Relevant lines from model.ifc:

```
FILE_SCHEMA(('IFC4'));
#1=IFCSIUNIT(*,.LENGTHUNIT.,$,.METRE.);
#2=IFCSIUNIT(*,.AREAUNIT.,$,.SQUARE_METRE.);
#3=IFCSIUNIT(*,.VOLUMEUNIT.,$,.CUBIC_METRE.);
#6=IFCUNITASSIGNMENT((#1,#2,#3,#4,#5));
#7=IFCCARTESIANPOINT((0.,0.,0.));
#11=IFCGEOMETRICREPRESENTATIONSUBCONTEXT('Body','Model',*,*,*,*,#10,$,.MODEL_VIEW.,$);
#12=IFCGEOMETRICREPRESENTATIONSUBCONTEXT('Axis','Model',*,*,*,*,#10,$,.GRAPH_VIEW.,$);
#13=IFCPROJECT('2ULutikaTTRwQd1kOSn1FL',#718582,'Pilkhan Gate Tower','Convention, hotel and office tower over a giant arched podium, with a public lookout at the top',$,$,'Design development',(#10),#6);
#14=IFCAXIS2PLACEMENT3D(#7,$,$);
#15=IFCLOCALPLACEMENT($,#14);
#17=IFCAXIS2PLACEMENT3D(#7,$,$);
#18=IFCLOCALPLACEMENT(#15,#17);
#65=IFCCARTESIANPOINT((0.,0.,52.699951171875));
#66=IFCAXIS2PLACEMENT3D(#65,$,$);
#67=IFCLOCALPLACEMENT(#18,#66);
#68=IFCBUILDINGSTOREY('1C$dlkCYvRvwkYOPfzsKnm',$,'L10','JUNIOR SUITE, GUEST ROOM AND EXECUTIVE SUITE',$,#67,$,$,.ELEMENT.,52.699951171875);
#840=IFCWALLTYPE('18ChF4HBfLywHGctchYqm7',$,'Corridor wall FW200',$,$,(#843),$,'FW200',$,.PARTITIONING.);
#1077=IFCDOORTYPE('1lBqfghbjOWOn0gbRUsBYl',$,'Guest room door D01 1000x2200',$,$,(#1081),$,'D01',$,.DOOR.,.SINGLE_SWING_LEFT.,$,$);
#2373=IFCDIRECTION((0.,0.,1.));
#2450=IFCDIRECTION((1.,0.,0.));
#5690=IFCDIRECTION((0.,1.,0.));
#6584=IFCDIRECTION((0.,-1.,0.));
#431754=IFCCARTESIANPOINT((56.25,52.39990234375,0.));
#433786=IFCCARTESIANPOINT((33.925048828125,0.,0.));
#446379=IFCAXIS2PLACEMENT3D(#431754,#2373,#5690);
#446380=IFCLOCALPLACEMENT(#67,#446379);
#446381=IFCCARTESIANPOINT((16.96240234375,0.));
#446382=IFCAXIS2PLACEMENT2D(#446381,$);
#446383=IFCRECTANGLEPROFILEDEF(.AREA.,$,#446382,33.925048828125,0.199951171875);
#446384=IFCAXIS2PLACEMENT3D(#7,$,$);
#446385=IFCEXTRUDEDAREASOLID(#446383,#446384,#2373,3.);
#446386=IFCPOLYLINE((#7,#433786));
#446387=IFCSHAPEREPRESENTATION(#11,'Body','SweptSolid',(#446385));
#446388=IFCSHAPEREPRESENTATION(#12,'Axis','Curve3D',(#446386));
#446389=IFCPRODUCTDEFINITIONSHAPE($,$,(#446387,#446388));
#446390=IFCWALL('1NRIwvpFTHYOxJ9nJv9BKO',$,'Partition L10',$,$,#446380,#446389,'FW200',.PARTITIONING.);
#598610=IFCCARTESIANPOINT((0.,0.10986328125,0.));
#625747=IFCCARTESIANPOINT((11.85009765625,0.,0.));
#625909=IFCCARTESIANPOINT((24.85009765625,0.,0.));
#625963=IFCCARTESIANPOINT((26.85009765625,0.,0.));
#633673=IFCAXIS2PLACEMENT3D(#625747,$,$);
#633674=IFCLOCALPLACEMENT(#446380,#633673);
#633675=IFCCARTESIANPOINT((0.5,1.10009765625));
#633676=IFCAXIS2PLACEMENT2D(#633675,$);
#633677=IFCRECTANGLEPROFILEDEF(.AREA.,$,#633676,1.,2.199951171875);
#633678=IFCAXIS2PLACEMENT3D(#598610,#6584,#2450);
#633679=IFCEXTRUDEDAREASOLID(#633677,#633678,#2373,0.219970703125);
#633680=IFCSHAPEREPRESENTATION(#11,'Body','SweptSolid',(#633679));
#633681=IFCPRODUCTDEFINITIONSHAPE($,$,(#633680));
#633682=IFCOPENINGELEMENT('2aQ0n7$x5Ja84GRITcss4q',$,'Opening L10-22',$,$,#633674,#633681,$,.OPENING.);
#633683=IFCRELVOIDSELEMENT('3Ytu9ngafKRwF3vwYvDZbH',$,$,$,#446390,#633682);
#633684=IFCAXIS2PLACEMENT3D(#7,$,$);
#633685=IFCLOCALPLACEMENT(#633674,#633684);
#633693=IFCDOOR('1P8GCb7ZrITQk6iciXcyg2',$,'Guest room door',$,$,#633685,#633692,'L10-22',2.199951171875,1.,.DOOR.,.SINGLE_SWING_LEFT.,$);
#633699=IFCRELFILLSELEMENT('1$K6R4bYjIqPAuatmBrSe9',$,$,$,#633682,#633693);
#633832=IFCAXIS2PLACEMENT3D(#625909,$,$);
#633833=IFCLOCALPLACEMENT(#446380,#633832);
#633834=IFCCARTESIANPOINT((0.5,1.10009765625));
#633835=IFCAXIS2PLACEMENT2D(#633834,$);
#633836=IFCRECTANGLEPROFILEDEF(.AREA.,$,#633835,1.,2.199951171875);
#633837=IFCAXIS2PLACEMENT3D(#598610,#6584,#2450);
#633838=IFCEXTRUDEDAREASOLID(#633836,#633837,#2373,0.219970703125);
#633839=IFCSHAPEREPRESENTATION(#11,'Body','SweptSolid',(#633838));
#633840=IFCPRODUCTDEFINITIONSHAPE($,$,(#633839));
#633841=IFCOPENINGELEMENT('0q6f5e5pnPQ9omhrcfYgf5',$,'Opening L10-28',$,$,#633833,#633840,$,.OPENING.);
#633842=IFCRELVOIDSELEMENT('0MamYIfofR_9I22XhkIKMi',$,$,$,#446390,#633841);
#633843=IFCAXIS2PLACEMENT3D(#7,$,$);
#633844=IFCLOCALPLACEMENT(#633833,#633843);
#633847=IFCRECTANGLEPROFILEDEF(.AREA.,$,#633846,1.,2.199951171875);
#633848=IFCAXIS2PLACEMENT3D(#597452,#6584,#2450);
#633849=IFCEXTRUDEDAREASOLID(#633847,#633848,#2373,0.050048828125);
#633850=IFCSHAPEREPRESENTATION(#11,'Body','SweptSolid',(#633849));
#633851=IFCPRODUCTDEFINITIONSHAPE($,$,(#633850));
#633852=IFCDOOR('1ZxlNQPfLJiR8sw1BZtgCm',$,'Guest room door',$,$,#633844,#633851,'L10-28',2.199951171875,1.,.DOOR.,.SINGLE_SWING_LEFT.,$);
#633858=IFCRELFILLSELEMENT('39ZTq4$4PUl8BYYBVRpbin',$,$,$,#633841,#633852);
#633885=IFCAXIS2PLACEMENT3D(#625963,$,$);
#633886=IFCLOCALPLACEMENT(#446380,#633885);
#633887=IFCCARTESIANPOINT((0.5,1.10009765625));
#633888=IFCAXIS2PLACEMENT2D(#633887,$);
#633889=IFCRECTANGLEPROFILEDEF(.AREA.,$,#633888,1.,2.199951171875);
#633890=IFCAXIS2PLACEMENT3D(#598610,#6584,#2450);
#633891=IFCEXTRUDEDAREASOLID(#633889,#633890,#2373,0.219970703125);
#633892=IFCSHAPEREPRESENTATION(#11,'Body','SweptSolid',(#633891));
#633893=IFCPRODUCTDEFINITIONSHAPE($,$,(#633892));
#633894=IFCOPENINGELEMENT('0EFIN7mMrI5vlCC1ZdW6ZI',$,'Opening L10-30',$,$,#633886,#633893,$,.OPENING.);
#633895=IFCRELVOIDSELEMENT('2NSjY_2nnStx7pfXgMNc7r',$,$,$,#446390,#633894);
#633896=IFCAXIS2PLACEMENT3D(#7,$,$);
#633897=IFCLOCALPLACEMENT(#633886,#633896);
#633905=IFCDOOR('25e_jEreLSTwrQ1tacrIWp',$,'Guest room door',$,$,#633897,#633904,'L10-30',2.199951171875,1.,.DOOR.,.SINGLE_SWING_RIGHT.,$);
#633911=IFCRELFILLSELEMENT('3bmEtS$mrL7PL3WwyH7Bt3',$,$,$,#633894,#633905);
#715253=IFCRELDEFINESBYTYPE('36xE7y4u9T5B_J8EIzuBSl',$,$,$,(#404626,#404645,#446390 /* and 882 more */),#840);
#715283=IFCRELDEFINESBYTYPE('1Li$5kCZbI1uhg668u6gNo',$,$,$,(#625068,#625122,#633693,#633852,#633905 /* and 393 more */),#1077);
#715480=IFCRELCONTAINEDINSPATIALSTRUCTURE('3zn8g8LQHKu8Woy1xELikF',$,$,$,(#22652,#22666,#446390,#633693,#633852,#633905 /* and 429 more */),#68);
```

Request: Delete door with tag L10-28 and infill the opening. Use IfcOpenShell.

```python
import ifcopenshell
import ifcopenshell.api.feature
import ifcopenshell.api.root
import ifcopenshell.geom
import ifcopenshell.util.shape

model = ifcopenshell.open("model.ifc")
settings = ifcopenshell.geom.settings()


def volume(element):
    """Net volume in cubic metres, openings subtracted."""
    shape = ifcopenshell.geom.create_shape(settings, element)
    return ifcopenshell.util.shape.get_volume(shape.geometry)


door = model.by_guid("1ZxlNQPfLJiR8sw1BZtgCm")
opening = door.FillsVoids[0].RelatingOpeningElement
wall = opening.VoidsElements[0].RelatingBuildingElement
before = volume(wall)

ifcopenshell.api.root.remove_product(model, product=door)
ifcopenshell.api.feature.remove_feature(model, feature=opening)

after = volume(wall)

print(f"wall volume {before:.3f} -> {after:.3f} m3")

model.write("model_rev.ifc")
```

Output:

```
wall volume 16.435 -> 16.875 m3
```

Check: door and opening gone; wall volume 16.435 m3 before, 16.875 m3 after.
